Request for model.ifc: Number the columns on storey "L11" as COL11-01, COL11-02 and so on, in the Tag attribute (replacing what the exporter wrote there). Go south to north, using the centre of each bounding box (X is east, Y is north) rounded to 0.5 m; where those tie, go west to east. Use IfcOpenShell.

First a look at what the model holds.

```python
import ifcopenshell
import ifcopenshell.util.element
import ifcopenshell.util.placement

model = ifcopenshell.open("model.ifc")
print(model.schema)
storey = next(s for s in model.by_type("IfcBuildingStorey") if s.Name == "L11")
columns = [e for e in ifcopenshell.util.element.get_decomposition(storey) if e.is_a("IfcColumn")]
for e in sorted(columns, key=lambda e: e.id()):
    origin = ifcopenshell.util.placement.get_local_placement(e.ObjectPlacement)[:3, 3]
    print(e.id(), e.Tag, e.Name, origin.round(2) + 0.0, sep=" | ")
```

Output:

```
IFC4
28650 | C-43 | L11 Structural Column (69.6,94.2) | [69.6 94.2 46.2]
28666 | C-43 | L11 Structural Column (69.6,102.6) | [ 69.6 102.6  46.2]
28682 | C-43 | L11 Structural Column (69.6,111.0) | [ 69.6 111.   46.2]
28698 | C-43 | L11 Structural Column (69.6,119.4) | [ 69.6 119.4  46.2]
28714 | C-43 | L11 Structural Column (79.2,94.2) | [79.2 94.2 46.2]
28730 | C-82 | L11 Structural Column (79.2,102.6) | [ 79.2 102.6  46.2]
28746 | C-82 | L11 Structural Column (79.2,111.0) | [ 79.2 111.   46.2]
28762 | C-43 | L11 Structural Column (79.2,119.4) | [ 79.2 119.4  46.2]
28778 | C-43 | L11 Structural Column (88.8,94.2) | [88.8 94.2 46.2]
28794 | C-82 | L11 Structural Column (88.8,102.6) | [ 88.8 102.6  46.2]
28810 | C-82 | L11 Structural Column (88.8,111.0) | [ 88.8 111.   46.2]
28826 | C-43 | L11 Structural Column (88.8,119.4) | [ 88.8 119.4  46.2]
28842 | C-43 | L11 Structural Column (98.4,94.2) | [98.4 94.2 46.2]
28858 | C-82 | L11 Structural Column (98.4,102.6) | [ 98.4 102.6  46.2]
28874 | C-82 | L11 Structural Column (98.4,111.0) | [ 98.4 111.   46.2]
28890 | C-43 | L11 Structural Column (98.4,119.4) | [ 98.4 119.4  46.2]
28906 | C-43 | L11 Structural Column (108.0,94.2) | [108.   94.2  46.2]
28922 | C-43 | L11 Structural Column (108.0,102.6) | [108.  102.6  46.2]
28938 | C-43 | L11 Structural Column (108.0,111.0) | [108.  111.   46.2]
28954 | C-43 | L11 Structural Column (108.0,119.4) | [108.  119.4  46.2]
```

```python
import ifcopenshell
import ifcopenshell.geom
import ifcopenshell.util.element
import ifcopenshell.util.shape

model = ifcopenshell.open("model.ifc")
settings = ifcopenshell.geom.settings()
settings.set("use-world-coords", True)


def centre(element):
    shape = ifcopenshell.geom.create_shape(settings, element)
    return ifcopenshell.util.shape.get_bbox_centroid(shape.geometry)


storey = next(s for s in model.by_type("IfcBuildingStorey") if s.Name == "L11")
columns = [e for e in ifcopenshell.util.element.get_decomposition(storey) if e.is_a("IfcColumn")]

# Insertion points can sit at a corner or the storey origin, so sort by the geometry (in metres).
centres = {e: centre(e) for e in columns}
columns.sort(key=lambda e: (round(centres[e][1] / 0.5), centres[e][0]))

for i, e in enumerate(columns, start=1):
    number = f"COL11-{i:02d}"
    e.Tag = number
    print(e.id(), number)

model.write("model_v2.ifc")
```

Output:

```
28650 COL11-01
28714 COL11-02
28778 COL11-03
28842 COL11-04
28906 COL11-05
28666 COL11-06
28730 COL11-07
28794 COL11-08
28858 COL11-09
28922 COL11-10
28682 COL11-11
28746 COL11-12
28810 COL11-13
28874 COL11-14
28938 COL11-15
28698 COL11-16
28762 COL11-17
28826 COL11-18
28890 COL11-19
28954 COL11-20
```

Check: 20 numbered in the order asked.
